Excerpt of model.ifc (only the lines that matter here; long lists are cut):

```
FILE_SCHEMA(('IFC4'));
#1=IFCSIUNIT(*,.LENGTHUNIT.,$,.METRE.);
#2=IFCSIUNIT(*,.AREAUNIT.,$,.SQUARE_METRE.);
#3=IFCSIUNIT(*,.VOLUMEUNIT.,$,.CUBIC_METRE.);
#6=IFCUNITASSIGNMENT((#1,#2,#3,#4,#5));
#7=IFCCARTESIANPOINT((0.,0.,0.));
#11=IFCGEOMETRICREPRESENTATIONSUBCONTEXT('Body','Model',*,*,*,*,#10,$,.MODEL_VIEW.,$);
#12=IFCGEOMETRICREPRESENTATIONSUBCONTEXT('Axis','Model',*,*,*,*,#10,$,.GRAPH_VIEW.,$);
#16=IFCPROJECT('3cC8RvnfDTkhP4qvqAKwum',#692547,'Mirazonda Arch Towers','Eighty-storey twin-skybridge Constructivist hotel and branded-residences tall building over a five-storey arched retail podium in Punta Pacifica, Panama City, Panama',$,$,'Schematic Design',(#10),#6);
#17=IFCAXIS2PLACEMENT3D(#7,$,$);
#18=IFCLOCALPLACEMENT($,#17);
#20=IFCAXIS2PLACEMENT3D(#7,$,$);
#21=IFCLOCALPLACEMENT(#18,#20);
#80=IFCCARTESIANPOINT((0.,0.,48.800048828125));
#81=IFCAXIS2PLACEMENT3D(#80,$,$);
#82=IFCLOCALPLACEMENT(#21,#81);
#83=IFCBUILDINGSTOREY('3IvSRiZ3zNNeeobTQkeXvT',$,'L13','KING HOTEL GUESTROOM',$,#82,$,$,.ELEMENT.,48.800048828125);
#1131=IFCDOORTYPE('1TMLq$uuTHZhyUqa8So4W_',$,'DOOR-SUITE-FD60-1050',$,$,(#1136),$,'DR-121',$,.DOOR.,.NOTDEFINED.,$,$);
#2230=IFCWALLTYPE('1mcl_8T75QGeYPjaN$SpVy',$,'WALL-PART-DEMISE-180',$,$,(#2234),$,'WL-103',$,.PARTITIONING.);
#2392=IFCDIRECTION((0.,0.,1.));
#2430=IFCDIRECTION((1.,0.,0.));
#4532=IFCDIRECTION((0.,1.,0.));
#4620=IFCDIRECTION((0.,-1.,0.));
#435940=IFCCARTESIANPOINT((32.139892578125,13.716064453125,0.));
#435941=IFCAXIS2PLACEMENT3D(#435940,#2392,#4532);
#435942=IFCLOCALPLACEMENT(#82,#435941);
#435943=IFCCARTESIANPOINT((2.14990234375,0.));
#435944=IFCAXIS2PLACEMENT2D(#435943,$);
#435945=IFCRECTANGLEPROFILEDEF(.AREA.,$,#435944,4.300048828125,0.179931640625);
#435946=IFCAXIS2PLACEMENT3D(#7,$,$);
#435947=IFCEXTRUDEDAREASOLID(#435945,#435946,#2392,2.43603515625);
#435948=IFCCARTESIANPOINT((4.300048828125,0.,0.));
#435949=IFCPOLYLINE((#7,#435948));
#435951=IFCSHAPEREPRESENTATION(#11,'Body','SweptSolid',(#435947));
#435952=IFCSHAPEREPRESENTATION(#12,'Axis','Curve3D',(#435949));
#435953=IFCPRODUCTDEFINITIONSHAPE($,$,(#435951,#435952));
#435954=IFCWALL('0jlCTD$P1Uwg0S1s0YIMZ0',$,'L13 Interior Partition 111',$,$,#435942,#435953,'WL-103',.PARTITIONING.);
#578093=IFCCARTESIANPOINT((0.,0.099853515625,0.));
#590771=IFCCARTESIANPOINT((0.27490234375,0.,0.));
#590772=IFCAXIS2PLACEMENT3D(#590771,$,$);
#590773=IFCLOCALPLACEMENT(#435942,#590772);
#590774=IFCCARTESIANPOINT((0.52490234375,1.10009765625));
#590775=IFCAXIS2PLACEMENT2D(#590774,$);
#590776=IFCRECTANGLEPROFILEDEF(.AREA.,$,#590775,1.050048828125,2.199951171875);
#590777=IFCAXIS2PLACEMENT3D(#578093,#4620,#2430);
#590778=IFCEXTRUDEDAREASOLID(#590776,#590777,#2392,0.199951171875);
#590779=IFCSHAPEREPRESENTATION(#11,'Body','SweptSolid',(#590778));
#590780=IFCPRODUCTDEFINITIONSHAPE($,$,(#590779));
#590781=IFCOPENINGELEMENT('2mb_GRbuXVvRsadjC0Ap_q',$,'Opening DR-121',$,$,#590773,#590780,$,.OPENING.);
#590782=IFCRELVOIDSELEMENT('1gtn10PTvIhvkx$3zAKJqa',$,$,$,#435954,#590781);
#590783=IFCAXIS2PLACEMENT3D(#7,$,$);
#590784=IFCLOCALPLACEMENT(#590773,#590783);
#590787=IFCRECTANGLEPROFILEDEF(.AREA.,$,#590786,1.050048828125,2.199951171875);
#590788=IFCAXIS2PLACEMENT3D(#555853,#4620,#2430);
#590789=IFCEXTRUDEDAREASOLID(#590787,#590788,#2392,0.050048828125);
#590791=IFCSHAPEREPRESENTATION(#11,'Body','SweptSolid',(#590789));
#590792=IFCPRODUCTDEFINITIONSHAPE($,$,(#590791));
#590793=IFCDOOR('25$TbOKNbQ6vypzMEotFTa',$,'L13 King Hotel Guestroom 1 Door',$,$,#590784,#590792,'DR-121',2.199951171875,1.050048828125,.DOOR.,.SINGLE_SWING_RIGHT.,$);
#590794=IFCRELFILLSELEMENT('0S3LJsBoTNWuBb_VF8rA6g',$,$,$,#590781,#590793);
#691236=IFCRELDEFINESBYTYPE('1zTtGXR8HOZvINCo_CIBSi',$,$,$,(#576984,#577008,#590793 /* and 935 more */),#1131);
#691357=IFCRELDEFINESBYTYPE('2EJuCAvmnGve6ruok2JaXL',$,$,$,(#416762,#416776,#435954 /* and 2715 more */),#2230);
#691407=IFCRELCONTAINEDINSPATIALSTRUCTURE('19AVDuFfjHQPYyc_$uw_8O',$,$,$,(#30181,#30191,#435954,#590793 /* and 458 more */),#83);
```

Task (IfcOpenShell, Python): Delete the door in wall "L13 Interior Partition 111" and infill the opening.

```python
import ifcopenshell
import ifcopenshell.api.feature
import ifcopenshell.api.root
import ifcopenshell.geom
import ifcopenshell.util.shape

model = ifcopenshell.open("model.ifc")
settings = ifcopenshell.geom.settings()


def volume(element):
    """Net volume in cubic metres, openings subtracted."""
    shape = ifcopenshell.geom.create_shape(settings, element)
    return ifcopenshell.util.shape.get_volume(shape.geometry)


door = model.by_guid("25$TbOKNbQ6vypzMEotFTa")
opening = door.FillsVoids[0].RelatingOpeningElement
wall = opening.VoidsElements[0].RelatingBuildingElement
before = volume(wall)

ifcopenshell.api.root.remove_product(model, product=door)
ifcopenshell.api.feature.remove_feature(model, feature=opening)

after = volume(wall)

print(f"wall volume {before:.3f} -> {after:.3f} m3")

model.write("model_rev.ifc")
```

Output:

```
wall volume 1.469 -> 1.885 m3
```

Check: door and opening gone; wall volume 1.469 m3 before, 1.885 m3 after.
